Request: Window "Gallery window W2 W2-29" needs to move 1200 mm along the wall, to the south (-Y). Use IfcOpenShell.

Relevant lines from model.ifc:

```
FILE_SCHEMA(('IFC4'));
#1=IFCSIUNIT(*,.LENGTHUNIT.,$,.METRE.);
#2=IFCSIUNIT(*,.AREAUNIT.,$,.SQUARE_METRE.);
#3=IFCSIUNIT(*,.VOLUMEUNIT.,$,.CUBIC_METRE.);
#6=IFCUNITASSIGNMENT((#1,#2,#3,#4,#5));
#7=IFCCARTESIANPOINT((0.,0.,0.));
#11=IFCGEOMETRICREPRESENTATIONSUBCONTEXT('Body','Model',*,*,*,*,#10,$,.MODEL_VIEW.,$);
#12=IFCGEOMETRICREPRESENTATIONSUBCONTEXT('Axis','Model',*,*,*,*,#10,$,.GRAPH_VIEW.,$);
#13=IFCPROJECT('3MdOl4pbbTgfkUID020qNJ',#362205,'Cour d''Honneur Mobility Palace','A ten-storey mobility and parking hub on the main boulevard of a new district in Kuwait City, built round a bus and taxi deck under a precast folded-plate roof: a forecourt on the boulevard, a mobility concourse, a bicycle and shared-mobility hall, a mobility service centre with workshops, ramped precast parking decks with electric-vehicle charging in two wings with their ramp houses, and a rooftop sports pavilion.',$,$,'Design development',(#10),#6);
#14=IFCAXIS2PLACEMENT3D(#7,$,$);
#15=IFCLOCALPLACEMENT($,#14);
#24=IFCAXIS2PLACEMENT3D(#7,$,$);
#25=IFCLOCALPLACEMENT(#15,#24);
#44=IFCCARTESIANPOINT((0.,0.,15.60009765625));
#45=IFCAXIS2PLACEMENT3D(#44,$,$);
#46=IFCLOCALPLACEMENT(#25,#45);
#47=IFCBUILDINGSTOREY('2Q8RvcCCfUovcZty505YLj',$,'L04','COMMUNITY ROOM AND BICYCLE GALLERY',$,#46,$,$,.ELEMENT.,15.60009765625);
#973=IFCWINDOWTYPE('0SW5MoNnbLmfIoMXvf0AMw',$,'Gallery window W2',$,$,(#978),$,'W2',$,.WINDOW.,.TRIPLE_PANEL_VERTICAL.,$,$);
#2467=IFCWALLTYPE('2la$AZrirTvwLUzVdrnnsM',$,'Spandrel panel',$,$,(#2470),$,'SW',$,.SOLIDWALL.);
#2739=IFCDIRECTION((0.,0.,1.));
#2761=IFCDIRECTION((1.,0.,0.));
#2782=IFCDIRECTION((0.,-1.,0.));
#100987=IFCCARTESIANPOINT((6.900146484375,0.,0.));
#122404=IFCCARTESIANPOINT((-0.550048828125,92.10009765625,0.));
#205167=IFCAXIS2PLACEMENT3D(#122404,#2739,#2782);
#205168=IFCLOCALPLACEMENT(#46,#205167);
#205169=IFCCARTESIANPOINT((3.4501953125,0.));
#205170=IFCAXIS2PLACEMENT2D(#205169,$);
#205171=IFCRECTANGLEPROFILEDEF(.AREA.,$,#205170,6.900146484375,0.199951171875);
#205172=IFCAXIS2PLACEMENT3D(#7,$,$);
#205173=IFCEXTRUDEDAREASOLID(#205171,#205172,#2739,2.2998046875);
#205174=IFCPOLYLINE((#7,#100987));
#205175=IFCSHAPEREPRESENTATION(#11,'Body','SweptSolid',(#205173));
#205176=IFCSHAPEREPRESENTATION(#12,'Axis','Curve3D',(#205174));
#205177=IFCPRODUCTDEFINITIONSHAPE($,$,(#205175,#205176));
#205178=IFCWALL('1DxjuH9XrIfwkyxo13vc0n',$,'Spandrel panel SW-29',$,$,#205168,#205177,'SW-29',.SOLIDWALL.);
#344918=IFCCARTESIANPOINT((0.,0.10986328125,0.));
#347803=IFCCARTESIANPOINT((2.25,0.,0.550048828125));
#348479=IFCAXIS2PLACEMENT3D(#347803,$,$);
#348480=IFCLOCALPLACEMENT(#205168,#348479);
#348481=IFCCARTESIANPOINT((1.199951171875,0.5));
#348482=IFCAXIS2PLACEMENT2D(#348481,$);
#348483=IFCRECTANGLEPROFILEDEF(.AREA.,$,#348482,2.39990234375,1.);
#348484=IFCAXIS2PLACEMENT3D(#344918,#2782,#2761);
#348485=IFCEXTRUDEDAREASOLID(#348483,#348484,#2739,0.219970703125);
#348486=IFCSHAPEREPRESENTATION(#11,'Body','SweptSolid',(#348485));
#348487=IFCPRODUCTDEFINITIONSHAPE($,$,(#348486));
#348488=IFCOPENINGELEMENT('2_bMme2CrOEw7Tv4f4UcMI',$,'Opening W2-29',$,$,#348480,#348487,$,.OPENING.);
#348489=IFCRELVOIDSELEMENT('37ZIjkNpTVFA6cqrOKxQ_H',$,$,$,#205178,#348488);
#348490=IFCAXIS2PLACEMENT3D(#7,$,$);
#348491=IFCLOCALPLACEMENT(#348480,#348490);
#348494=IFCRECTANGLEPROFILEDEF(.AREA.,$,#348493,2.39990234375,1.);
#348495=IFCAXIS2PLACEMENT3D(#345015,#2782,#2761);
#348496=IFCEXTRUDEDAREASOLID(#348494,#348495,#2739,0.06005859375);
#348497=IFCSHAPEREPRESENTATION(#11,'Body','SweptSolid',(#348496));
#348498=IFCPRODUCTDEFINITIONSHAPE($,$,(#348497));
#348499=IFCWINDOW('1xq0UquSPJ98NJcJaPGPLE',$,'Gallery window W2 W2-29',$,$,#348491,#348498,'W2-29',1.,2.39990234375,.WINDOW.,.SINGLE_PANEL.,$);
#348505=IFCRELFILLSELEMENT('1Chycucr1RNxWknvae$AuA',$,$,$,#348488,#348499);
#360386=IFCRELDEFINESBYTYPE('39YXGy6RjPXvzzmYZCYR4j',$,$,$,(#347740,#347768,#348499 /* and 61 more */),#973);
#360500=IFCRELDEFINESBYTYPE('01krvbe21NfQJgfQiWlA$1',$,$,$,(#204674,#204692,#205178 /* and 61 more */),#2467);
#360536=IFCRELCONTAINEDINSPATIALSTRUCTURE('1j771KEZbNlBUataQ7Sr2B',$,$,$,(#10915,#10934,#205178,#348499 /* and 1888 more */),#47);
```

```python
import ifcopenshell
import ifcopenshell.api.geometry
import ifcopenshell.util.placement
import ifcopenshell.util.unit

model = ifcopenshell.open("model.ifc")
unit_scale = ifcopenshell.util.unit.calculate_unit_scale(model)

window = model.by_guid("1xq0UquSPJ98NJcJaPGPLE")
opening = window.FillsVoids[0].RelatingOpeningElement
wall = opening.VoidsElements[0].RelatingBuildingElement

wall_matrix = ifcopenshell.util.placement.get_local_placement(wall.ObjectPlacement)
shift = wall_matrix[:3, 0] * 1.2 / unit_scale
before = ifcopenshell.util.placement.get_local_placement(window.ObjectPlacement)[:3, 3].copy()

# The window is placed relative to its opening, so it follows when the opening moves.
matrix = ifcopenshell.util.placement.get_local_placement(opening.ObjectPlacement)
matrix[:3, 3] += shift
ifcopenshell.api.geometry.edit_object_placement(
    model, product=opening, matrix=matrix, is_si=False, should_transform_children=True
)

after = ifcopenshell.util.placement.get_local_placement(window.ObjectPlacement)[:3, 3]
print("window moved by", (after - before).round(3) + 0.0)

model.write("model-out.ifc")
```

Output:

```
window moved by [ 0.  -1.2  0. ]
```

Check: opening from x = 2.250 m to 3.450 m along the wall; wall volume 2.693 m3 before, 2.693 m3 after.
